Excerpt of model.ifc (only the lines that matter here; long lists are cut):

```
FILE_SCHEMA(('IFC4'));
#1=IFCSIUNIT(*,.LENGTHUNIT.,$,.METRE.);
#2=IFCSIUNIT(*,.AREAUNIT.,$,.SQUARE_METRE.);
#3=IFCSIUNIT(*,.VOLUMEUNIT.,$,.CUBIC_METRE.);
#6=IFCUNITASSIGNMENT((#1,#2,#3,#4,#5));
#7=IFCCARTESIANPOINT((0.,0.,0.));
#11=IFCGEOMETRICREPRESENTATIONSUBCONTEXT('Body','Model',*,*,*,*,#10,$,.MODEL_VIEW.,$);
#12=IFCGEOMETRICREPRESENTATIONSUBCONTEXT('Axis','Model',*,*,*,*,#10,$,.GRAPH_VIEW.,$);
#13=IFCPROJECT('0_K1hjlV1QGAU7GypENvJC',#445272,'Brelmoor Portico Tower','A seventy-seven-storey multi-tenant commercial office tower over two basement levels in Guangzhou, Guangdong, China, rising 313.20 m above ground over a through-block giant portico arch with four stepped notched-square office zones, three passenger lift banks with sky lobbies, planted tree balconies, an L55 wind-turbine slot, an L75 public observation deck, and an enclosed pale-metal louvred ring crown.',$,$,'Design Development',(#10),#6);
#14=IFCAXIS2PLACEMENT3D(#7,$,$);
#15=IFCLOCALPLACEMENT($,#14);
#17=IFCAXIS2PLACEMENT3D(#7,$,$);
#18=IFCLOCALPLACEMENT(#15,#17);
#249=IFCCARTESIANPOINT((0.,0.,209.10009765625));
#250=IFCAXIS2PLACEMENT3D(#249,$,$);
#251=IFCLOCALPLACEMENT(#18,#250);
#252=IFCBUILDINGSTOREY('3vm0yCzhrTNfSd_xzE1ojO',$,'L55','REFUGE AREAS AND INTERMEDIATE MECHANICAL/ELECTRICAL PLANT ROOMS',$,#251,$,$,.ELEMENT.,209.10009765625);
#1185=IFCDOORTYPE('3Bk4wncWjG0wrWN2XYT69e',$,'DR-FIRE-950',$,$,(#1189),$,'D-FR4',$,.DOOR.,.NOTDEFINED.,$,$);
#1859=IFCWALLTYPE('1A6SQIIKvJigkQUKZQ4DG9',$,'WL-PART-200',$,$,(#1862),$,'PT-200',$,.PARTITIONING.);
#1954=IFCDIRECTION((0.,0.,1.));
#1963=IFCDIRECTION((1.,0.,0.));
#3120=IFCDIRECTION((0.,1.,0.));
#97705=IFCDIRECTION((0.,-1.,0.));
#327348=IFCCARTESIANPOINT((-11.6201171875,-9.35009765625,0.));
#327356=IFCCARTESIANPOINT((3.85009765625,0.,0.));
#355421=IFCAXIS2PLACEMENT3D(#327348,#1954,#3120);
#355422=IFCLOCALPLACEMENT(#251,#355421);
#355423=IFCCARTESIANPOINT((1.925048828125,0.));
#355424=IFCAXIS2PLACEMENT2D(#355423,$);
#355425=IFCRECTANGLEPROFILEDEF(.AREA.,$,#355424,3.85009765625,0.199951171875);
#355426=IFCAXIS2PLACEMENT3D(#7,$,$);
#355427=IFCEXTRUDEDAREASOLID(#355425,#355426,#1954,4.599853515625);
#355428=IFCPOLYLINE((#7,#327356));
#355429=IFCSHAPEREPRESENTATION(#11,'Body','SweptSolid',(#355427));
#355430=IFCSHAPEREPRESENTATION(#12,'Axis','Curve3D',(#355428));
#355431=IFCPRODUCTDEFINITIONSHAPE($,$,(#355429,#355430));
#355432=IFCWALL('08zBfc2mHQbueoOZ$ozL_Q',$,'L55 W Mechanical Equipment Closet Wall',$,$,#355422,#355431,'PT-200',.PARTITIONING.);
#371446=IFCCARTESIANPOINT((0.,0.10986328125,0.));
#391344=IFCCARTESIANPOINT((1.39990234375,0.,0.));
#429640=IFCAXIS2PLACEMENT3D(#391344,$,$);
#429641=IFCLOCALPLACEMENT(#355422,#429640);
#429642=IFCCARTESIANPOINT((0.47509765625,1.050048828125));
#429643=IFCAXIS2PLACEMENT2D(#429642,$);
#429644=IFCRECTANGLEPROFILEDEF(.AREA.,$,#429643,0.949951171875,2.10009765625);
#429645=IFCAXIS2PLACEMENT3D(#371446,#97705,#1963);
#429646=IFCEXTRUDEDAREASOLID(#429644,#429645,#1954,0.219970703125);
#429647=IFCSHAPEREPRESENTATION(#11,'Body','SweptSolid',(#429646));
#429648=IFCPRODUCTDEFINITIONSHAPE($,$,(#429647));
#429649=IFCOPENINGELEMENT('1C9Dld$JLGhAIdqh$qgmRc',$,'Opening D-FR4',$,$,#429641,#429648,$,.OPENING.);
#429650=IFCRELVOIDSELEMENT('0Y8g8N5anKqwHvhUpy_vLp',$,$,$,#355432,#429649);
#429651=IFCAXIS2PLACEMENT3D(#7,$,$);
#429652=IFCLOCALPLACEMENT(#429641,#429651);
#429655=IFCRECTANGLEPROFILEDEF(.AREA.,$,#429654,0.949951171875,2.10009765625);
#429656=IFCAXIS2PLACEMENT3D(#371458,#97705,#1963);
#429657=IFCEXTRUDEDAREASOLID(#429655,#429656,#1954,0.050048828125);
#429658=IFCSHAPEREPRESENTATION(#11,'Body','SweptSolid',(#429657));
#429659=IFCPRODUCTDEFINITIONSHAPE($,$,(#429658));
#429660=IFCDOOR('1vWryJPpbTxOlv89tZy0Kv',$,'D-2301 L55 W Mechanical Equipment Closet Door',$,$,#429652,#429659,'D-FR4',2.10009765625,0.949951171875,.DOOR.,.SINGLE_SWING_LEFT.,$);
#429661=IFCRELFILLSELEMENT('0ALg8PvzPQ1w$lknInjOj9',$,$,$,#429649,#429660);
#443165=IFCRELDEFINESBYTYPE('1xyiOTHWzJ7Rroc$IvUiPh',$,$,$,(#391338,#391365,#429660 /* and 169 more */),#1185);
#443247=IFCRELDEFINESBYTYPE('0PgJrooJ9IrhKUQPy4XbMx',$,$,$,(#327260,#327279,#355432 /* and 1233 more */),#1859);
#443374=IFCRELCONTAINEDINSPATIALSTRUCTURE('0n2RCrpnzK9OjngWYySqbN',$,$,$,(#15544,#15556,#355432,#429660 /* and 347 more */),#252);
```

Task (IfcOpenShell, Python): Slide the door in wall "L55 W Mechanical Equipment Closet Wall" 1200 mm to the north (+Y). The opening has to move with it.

```python
import ifcopenshell
import ifcopenshell.api.geometry
import ifcopenshell.util.placement
import ifcopenshell.util.unit

model = ifcopenshell.open("model.ifc")
unit_scale = ifcopenshell.util.unit.calculate_unit_scale(model)

door = model.by_guid("1vWryJPpbTxOlv89tZy0Kv")
opening = door.FillsVoids[0].RelatingOpeningElement
wall = opening.VoidsElements[0].RelatingBuildingElement

wall_matrix = ifcopenshell.util.placement.get_local_placement(wall.ObjectPlacement)
shift = wall_matrix[:3, 0] * 1.2 / unit_scale
before = ifcopenshell.util.placement.get_local_placement(door.ObjectPlacement)[:3, 3].copy()

# The door is placed relative to its opening, so it follows when the opening moves.
matrix = ifcopenshell.util.placement.get_local_placement(opening.ObjectPlacement)
matrix[:3, 3] += shift
ifcopenshell.api.geometry.edit_object_placement(
    model, product=opening, matrix=matrix, is_si=False, should_transform_children=True
)

after = ifcopenshell.util.placement.get_local_placement(door.ObjectPlacement)[:3, 3]
print("door moved by", (after - before).round(3) + 0.0)

model.write("model_rev.ifc")
```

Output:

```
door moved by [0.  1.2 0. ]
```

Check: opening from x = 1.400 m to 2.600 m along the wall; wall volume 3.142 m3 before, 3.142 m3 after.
